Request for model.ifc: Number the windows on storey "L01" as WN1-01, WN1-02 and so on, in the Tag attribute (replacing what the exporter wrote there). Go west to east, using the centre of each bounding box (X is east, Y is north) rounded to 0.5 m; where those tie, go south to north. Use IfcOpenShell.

First a look at what the model holds.

```python
import ifcopenshell
import ifcopenshell.util.element
import ifcopenshell.util.placement

model = ifcopenshell.open("model.ifc")
print(model.schema)
storey = next(s for s in model.by_type("IfcBuildingStorey") if s.Name == "L01")
windows = [e for e in ifcopenshell.util.element.get_decomposition(storey) if e.is_a("IfcWindow")]
for e in sorted(windows, key=lambda e: e.id()):
    origin = ifcopenshell.util.placement.get_local_placement(e.ObjectPlacement)[:3, 3]
    print(e.id(), e.Tag, e.Name, origin.round(2) + 0.0, sep=" | ")
```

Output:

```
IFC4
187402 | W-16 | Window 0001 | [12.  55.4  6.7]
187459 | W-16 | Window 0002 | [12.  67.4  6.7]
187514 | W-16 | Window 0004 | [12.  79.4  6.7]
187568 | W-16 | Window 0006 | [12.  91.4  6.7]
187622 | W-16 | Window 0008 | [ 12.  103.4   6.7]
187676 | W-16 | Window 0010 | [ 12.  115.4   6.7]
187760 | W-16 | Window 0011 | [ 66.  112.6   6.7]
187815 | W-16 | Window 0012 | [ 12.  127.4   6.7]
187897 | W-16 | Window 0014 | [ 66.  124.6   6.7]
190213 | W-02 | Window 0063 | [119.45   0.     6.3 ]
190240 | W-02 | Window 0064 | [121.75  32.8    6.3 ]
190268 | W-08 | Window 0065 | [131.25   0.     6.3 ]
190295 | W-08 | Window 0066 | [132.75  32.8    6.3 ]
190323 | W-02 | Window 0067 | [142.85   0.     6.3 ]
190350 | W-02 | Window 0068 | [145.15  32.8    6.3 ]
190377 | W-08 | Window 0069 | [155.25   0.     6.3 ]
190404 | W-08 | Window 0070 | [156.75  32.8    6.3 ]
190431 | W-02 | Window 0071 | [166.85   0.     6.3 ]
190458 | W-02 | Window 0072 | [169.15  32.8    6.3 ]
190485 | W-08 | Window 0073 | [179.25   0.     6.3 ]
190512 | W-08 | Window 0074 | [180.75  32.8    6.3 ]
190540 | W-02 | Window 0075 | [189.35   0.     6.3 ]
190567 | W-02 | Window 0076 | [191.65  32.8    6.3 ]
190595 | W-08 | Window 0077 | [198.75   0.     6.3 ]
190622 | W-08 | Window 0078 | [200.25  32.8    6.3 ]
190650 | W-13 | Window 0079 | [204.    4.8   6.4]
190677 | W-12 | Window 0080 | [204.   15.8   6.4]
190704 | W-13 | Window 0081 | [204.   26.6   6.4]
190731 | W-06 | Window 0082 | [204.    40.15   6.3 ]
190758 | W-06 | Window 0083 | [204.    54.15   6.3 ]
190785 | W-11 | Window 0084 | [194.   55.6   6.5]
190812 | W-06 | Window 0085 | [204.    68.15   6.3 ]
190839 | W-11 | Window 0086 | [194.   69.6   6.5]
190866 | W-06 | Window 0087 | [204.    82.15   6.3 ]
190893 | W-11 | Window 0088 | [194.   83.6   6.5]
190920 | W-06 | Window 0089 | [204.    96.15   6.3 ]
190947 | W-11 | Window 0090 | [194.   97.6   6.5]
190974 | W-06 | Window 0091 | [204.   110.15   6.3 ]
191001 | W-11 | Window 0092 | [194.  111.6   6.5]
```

```python
import ifcopenshell
import ifcopenshell.geom
import ifcopenshell.util.element
import ifcopenshell.util.shape

model = ifcopenshell.open("model.ifc")
settings = ifcopenshell.geom.settings()
settings.set("use-world-coords", True)


def centre(element):
    shape = ifcopenshell.geom.create_shape(settings, element)
    return ifcopenshell.util.shape.get_bbox_centroid(shape.geometry)


storey = next(s for s in model.by_type("IfcBuildingStorey") if s.Name == "L01")
windows = [e for e in ifcopenshell.util.element.get_decomposition(storey) if e.is_a("IfcWindow")]

# Insertion points can sit at a corner or the storey origin, so sort by the geometry (in metres).
centres = {e: centre(e) for e in windows}
windows.sort(key=lambda e: (round(centres[e][0] / 0.5), centres[e][1]))

for i, e in enumerate(windows, start=1):
    number = f"WN1-{i:02d}"
    e.Tag = number
    print(e.id(), number)

model.write("model-out.ifc")
```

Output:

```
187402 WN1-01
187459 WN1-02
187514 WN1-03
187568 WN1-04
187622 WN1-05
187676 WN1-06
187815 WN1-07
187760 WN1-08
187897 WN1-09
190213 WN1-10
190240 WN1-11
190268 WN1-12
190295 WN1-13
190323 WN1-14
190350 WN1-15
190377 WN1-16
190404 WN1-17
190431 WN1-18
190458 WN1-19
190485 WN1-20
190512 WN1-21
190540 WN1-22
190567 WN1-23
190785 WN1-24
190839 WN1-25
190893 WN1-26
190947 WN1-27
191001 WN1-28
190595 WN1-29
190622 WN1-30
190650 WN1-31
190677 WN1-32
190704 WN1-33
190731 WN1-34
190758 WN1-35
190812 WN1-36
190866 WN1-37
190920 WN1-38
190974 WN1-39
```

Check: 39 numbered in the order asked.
